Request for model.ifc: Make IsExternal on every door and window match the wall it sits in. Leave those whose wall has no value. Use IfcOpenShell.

First a look at what the model holds.

```python
import ifcopenshell
import ifcopenshell.util.element

model = ifcopenshell.open("model.ifc")
print(model.schema)
seen = {}
for e in model.by_type("IfcDoor") + model.by_type("IfcWindow"):
    if not e.FillsVoids:
        continue
    host = e.FillsVoids[0].RelatingOpeningElement.VoidsElements[0].RelatingBuildingElement
    own = ifcopenshell.util.element.get_pset(e, f"Pset_{e.is_a()[3:].removesuffix('StandardCase')}Common", "IsExternal")
    wall = ifcopenshell.util.element.get_pset(host, "Pset_WallCommon", "IsExternal")
    seen[e.is_a(), own, wall] = seen.get((e.is_a(), own, wall), 0) + 1
for (cls, own, wall), count in sorted(seen.items(), key=str):
    print(count, cls, "IsExternal:", own, "| host wall:", wall)
```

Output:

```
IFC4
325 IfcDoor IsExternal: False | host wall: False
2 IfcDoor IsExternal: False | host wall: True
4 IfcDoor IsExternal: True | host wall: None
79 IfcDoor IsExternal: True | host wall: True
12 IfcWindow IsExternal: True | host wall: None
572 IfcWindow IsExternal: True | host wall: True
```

```python
import ifcopenshell
import ifcopenshell.api.pset
import ifcopenshell.util.element

model = ifcopenshell.open("model.ifc")

count = 0
for ifc_class, pset_name in (("IfcDoor", "Pset_DoorCommon"), ("IfcWindow", "Pset_WindowCommon")):
    for e in model.by_type(ifc_class):
        if not e.FillsVoids:
            continue
        host = e.FillsVoids[0].RelatingOpeningElement.VoidsElements[0].RelatingBuildingElement
        external = ifcopenshell.util.element.get_pset(host, "Pset_WallCommon", "IsExternal")
        if external is None or ifcopenshell.util.element.get_pset(e, pset_name, "IsExternal") == external:
            continue
        pset = ifcopenshell.api.pset.add_pset(model, product=e, name=pset_name)
        ifcopenshell.api.pset.edit_pset(model, pset=pset, properties={"IsExternal": external})
        count += 1

print(count, "updated")

model.write("model_rev.ifc")
```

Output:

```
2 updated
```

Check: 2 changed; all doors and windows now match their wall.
